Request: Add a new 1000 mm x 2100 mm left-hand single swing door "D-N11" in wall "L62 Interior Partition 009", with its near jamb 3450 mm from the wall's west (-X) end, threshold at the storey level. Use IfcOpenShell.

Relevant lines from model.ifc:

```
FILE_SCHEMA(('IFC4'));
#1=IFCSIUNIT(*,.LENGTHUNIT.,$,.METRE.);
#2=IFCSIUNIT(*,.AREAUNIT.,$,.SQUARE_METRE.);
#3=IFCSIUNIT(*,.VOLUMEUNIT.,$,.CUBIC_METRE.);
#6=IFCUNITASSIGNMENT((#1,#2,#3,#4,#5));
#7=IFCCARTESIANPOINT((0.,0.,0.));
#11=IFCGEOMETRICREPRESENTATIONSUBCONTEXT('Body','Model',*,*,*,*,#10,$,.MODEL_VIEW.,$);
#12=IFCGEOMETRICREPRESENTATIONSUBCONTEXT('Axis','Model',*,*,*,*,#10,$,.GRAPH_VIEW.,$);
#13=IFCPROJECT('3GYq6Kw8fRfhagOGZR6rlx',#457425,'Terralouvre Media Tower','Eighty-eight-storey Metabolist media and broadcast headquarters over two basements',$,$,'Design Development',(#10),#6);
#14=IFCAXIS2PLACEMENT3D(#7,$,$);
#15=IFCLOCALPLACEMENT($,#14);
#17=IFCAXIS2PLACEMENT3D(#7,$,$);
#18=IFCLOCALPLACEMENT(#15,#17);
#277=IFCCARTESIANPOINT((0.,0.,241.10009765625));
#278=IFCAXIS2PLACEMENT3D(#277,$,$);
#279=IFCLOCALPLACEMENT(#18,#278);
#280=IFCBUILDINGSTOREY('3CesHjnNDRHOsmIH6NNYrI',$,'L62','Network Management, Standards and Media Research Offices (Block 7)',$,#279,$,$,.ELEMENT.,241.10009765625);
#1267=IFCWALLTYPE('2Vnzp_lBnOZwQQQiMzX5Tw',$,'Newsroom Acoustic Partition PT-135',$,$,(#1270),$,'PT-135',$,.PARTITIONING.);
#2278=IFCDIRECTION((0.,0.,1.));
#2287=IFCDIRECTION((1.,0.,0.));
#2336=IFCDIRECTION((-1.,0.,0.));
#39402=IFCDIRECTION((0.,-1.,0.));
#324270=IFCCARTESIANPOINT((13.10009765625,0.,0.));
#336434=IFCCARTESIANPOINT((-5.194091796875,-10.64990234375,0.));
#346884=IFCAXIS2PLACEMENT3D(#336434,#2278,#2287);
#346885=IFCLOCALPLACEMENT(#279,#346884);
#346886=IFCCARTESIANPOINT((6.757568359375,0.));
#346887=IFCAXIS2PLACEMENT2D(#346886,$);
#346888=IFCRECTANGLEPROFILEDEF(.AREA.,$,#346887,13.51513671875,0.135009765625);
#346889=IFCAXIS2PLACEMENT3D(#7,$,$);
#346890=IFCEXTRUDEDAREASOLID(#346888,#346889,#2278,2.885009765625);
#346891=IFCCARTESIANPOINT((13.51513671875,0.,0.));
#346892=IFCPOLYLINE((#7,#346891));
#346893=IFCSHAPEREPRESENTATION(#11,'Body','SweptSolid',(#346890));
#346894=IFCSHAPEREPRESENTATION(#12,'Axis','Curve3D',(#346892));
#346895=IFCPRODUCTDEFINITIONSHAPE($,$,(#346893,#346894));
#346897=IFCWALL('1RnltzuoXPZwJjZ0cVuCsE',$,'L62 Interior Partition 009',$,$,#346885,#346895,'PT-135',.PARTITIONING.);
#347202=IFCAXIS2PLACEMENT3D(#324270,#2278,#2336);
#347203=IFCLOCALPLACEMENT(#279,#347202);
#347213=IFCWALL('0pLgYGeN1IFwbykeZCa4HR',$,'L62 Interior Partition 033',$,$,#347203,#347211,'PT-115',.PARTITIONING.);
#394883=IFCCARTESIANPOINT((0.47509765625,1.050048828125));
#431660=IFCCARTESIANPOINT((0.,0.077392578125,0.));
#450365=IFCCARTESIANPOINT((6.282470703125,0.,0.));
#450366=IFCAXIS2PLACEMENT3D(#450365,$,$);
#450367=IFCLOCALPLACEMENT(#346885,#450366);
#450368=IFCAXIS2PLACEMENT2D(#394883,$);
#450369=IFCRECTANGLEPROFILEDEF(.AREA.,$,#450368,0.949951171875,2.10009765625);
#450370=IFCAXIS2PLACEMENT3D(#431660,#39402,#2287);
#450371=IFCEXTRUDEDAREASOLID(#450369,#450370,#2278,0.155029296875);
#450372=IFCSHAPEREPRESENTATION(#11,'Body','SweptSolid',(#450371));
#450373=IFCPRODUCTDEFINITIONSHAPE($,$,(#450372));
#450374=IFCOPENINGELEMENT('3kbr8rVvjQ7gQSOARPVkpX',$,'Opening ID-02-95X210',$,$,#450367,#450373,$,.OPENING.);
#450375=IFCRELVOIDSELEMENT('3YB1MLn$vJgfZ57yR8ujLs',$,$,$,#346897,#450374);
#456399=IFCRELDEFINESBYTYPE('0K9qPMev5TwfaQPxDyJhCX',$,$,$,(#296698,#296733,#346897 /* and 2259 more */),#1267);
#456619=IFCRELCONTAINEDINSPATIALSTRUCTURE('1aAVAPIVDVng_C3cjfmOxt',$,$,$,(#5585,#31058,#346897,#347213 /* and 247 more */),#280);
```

```python
import numpy as np
import ifcopenshell
import ifcopenshell.api.feature
import ifcopenshell.api.geometry
import ifcopenshell.api.root
import ifcopenshell.api.spatial
import ifcopenshell.geom
import ifcopenshell.util.element
import ifcopenshell.util.placement
import ifcopenshell.util.representation
import ifcopenshell.util.shape
import ifcopenshell.util.unit

model = ifcopenshell.open("model.ifc")
unit_scale = ifcopenshell.util.unit.calculate_unit_scale(model)
settings = ifcopenshell.geom.settings()


def volume(element):
    """Net volume in cubic metres, openings subtracted."""
    shape = ifcopenshell.geom.create_shape(settings, element)
    return ifcopenshell.util.shape.get_volume(shape.geometry)


wall = model.by_guid("1RnltzuoXPZwJjZ0cVuCsE")
storey = ifcopenshell.util.element.get_container(wall, ifc_class="IfcBuildingStorey")
context = ifcopenshell.util.representation.get_context(model, "Model", "Body", "MODEL_VIEW")
before = volume(wall)

width, height, from_end, sill = 1, 2.1, 3.45, 0.0  # metres

# The wall runs along its own X axis, and the end named is its -X end.
wall_shape = ifcopenshell.geom.create_shape(settings, wall)
x, y, z = ifcopenshell.util.shape.get_vertices(wall_shape.geometry).T
start = x.min() + from_end
face, thickness = float(y.min()), float(y.max() - y.min())
wall_matrix = ifcopenshell.util.placement.get_local_placement(wall.ObjectPlacement)
level = ifcopenshell.util.placement.get_local_placement(storey.ObjectPlacement)[2, 3]


def in_wall(x, y):
    """Placement at x, y metres in the wall's axes, at sill height."""
    matrix = wall_matrix.copy()
    matrix[:, 3] = wall_matrix @ np.array([x / unit_scale, y / unit_scale, 0.0, 1.0])
    matrix[2, 3] = level + sill / unit_scale
    return matrix


# Opening: a box that overshoots both wall faces by 50 mm.
opening = ifcopenshell.api.root.create_entity(model, ifc_class="IfcOpeningElement", predefined_type="OPENING")
box = ifcopenshell.api.geometry.add_wall_representation(
    model, context=context, length=width, height=height, thickness=thickness + 0.1
)
ifcopenshell.api.geometry.assign_representation(model, product=opening, representation=box)
ifcopenshell.api.geometry.edit_object_placement(model, product=opening, matrix=in_wall(start, face - 0.05), is_si=False)
ifcopenshell.api.feature.add_feature(model, feature=opening, element=wall)

door = ifcopenshell.api.root.create_entity(model, ifc_class="IfcDoor", name="D-N11", predefined_type="DOOR")
door.OverallWidth, door.OverallHeight = width / unit_scale, height / unit_scale
door.OperationType = "SINGLE_SWING_LEFT"
body = ifcopenshell.api.geometry.add_door_representation(
    model,
    context=context,
    overall_width=door.OverallWidth,
    overall_height=door.OverallHeight,
    operation_type="SINGLE_SWING_LEFT",
    lining_properties={"LiningDepth": thickness / unit_scale, "ThresholdDepth": thickness / unit_scale},
)
ifcopenshell.api.geometry.assign_representation(model, product=door, representation=body)
ifcopenshell.api.spatial.assign_container(model, products=[door], relating_structure=storey)
ifcopenshell.api.feature.add_filling(model, opening=opening, element=door)

# The lining spans the wall, so the door starts at the wall face.
ifcopenshell.api.geometry.edit_object_placement(model, product=door, matrix=in_wall(start, face), is_si=False)

after = volume(wall)

print(f"wall volume {before:.3f} -> {after:.3f} m3")

model.write("model_edited.ifc")
```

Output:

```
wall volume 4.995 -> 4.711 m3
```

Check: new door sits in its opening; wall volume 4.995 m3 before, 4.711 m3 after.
